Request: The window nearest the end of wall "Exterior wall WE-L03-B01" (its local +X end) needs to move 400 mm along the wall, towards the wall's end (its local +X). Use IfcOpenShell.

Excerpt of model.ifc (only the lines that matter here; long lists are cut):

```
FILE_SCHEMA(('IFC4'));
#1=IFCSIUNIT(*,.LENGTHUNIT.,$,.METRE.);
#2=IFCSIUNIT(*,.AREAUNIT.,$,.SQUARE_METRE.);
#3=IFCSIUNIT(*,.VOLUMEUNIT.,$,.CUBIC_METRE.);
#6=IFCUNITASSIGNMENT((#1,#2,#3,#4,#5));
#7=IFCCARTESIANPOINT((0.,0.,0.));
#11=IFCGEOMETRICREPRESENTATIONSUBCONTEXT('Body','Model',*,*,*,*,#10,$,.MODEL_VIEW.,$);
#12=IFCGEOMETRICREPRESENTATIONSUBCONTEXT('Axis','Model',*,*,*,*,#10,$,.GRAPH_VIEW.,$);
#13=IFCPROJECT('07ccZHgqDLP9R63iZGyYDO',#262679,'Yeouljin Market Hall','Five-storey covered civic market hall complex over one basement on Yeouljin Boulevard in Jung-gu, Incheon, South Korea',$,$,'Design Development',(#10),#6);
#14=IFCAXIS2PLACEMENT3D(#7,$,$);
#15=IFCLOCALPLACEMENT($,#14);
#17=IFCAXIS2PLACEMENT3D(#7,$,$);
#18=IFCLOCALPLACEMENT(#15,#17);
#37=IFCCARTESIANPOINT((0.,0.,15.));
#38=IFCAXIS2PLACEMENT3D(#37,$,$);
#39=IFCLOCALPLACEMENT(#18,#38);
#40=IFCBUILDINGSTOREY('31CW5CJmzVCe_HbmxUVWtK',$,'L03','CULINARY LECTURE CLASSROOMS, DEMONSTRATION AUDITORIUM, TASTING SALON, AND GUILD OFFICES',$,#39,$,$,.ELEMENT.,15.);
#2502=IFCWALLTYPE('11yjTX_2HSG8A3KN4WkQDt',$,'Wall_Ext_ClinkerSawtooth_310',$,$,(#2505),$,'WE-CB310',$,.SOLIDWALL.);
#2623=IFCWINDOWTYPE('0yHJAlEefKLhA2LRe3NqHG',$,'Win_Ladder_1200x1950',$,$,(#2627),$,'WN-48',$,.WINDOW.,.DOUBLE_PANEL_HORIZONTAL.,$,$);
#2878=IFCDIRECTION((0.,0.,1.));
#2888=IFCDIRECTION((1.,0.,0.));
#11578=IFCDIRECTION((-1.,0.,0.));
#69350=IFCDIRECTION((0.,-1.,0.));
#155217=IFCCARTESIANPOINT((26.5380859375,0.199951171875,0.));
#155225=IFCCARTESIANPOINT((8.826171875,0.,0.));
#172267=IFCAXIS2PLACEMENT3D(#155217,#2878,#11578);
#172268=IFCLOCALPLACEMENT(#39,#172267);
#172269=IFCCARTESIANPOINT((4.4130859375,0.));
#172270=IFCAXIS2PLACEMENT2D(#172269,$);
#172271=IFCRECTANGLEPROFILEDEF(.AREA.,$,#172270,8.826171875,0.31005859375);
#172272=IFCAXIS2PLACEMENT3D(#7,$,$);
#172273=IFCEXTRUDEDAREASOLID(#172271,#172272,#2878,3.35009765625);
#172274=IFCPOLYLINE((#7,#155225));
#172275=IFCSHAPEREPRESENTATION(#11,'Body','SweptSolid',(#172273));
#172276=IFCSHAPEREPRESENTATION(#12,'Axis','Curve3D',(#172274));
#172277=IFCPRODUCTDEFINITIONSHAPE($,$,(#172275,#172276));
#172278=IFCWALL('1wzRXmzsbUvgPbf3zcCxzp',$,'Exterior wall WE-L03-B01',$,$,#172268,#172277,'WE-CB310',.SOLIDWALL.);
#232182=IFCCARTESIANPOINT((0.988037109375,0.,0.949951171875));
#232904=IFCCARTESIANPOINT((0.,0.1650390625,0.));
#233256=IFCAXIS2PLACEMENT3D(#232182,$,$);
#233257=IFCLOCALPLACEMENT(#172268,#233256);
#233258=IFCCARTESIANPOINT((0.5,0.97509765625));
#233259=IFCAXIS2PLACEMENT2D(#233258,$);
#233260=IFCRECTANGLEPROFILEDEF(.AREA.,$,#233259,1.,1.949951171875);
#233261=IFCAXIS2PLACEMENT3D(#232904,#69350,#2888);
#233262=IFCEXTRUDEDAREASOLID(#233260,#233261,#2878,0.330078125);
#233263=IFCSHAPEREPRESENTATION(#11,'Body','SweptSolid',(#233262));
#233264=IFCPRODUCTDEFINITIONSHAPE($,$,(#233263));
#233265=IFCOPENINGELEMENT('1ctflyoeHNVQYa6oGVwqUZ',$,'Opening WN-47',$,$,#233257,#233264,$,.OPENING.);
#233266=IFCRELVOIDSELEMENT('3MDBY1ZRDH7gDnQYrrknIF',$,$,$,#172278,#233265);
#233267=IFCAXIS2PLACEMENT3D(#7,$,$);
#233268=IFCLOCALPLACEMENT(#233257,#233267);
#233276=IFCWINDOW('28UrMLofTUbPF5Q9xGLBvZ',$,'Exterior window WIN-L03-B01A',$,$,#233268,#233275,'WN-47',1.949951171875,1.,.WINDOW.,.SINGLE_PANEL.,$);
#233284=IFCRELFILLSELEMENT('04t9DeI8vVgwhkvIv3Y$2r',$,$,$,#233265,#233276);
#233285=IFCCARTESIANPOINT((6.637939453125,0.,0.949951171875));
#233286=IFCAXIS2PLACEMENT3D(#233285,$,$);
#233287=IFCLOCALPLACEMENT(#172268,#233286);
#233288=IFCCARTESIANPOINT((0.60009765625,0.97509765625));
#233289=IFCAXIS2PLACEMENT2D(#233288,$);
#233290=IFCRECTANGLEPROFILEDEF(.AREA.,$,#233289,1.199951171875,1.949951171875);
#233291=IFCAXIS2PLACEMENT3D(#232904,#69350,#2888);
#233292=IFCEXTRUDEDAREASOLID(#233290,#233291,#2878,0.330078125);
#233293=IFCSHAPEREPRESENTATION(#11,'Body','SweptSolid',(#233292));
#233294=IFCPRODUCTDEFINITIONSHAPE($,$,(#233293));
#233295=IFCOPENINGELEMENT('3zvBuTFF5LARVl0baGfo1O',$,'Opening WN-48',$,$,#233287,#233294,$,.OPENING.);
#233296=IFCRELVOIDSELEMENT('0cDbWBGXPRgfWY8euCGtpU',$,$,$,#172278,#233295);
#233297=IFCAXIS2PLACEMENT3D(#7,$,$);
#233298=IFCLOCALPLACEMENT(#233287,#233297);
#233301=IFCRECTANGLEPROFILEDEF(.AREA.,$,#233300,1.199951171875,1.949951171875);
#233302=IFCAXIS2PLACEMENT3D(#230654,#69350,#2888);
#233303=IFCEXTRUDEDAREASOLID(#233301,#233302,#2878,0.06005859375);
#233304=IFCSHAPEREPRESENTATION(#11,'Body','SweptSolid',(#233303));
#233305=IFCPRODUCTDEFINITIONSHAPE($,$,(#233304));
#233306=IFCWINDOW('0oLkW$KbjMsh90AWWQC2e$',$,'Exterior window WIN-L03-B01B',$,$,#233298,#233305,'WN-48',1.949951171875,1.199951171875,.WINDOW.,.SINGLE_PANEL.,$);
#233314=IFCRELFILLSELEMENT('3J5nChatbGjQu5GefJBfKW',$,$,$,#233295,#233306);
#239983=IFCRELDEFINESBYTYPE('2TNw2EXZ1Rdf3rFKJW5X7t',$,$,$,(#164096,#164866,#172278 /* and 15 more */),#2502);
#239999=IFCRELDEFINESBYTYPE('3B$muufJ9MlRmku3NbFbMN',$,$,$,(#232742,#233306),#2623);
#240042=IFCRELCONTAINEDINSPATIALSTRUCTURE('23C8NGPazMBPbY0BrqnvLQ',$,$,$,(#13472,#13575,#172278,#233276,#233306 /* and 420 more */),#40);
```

```python
import ifcopenshell
import ifcopenshell.api.geometry
import ifcopenshell.util.placement
import ifcopenshell.util.unit

model = ifcopenshell.open("model.ifc")
unit_scale = ifcopenshell.util.unit.calculate_unit_scale(model)

window = model.by_guid("0oLkW$KbjMsh90AWWQC2e$")
opening = window.FillsVoids[0].RelatingOpeningElement
wall = opening.VoidsElements[0].RelatingBuildingElement

wall_matrix = ifcopenshell.util.placement.get_local_placement(wall.ObjectPlacement)
shift = wall_matrix[:3, 0] * 0.4 / unit_scale
before = ifcopenshell.util.placement.get_local_placement(window.ObjectPlacement)[:3, 3].copy()

# The window is placed relative to its opening, so it follows when the opening moves.
matrix = ifcopenshell.util.placement.get_local_placement(opening.ObjectPlacement)
matrix[:3, 3] += shift
ifcopenshell.api.geometry.edit_object_placement(
    model, product=opening, matrix=matrix, is_si=False, should_transform_children=True
)

after = ifcopenshell.util.placement.get_local_placement(window.ObjectPlacement)[:3, 3]
print("window moved by", (after - before).round(3) + 0.0)

model.write("model_edited.ifc")
```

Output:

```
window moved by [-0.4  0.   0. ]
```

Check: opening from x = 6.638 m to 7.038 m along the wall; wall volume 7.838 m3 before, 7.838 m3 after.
